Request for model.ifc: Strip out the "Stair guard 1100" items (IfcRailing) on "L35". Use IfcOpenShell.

First a look at what the model holds.

```python
import ifcopenshell
import ifcopenshell.util.element

model = ifcopenshell.open("model.ifc")
print(model.schema)
storey = next(s for s in model.by_type("IfcBuildingStorey") if s.Name == "L35")
railings = [e for e in ifcopenshell.util.element.get_decomposition(storey) if e.is_a("IfcRailing")]
seen = {}
for e in railings:
    element_type = ifcopenshell.util.element.get_type(e)
    name = element_type.Name if element_type not in (None, e) else None
    seen[name] = seen.get(name, 0) + 1
for name, count in sorted(seen.items(), key=str):
    print(count, "x", name)
```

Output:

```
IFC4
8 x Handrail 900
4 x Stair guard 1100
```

```python
import ifcopenshell
import ifcopenshell.api.root
import ifcopenshell.util.element

model = ifcopenshell.open("model.ifc")

storey = next(s for s in model.by_type("IfcBuildingStorey") if s.Name == "L35")
railings = [e for e in ifcopenshell.util.element.get_decomposition(storey) if e.is_a("IfcRailing")]
targets = [e for e in railings if (t := ifcopenshell.util.element.get_type(e)) not in (None, e) and t.Name == "Stair guard 1100"]

for e in targets:
    ifcopenshell.api.root.remove_product(model, product=e)
print(len(targets), "removed")

model.write("model_v2.ifc")
```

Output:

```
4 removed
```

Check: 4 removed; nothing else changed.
